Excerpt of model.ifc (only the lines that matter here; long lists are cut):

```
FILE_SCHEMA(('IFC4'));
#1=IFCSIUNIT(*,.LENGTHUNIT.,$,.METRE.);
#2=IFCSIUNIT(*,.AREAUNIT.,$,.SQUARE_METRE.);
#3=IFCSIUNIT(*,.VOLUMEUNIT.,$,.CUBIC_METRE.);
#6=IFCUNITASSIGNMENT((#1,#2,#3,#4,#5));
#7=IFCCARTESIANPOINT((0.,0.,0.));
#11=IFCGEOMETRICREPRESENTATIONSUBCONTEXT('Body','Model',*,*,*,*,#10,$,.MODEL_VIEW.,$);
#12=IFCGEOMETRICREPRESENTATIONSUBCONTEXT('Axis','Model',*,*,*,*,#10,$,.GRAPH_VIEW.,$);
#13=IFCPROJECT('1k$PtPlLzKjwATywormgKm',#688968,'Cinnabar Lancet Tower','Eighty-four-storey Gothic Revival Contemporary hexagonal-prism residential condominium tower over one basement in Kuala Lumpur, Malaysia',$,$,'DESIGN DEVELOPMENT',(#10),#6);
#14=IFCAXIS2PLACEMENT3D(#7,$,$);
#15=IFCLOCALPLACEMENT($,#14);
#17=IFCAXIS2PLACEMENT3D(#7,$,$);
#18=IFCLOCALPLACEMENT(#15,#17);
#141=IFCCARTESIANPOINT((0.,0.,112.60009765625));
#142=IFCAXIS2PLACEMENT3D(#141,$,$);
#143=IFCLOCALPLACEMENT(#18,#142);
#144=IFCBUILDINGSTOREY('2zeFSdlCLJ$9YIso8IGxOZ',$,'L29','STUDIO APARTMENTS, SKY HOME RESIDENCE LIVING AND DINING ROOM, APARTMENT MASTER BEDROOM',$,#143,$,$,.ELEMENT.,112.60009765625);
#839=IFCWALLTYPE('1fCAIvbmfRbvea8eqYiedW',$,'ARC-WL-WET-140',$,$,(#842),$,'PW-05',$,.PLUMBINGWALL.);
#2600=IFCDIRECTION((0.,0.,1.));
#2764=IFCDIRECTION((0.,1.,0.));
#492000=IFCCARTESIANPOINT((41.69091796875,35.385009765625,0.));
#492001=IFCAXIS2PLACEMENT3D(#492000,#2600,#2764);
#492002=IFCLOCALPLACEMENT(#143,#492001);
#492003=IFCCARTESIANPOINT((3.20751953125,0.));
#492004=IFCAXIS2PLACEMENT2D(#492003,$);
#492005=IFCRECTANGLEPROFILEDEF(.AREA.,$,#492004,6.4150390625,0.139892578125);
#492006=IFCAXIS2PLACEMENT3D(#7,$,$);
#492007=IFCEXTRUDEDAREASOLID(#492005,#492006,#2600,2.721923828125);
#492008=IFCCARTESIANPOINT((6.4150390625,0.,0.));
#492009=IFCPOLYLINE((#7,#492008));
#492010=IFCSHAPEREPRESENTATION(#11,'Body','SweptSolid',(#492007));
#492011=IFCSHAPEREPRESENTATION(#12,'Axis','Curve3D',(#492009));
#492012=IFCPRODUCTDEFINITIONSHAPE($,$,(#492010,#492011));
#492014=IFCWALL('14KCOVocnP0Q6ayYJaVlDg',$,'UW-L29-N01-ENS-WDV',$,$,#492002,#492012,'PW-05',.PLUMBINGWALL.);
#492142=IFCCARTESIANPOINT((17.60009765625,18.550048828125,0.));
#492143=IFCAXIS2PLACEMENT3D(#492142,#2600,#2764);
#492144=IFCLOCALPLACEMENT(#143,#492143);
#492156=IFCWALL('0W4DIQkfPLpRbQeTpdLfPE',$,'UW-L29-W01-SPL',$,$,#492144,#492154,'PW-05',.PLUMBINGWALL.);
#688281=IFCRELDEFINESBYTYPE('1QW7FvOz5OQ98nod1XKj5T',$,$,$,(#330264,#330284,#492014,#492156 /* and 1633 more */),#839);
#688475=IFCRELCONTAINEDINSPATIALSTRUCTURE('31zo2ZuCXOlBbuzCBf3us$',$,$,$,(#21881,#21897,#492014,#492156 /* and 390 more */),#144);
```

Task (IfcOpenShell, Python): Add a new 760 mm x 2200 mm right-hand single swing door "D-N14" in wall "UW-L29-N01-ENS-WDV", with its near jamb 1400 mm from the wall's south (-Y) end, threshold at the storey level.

```python
import numpy as np
import ifcopenshell
import ifcopenshell.api.feature
import ifcopenshell.api.geometry
import ifcopenshell.api.root
import ifcopenshell.api.spatial
import ifcopenshell.geom
import ifcopenshell.util.element
import ifcopenshell.util.placement
import ifcopenshell.util.representation
import ifcopenshell.util.shape
import ifcopenshell.util.unit

model = ifcopenshell.open("model.ifc")
unit_scale = ifcopenshell.util.unit.calculate_unit_scale(model)
settings = ifcopenshell.geom.settings()


def volume(element):
    """Net volume in cubic metres, openings subtracted."""
    shape = ifcopenshell.geom.create_shape(settings, element)
    return ifcopenshell.util.shape.get_volume(shape.geometry)


wall = model.by_guid("14KCOVocnP0Q6ayYJaVlDg")
storey = ifcopenshell.util.element.get_container(wall, ifc_class="IfcBuildingStorey")
context = ifcopenshell.util.representation.get_context(model, "Model", "Body", "MODEL_VIEW")
before = volume(wall)

width, height, from_end, sill = 0.76, 2.2, 1.4, 0.0  # metres

# The wall runs along its own X axis, and the end named is its -X end.
wall_shape = ifcopenshell.geom.create_shape(settings, wall)
x, y, z = ifcopenshell.util.shape.get_vertices(wall_shape.geometry).T
start = x.min() + from_end
face, thickness = float(y.min()), float(y.max() - y.min())
wall_matrix = ifcopenshell.util.placement.get_local_placement(wall.ObjectPlacement)
level = ifcopenshell.util.placement.get_local_placement(storey.ObjectPlacement)[2, 3]


def in_wall(x, y):
    """Placement at x, y metres in the wall's axes, at sill height."""
    matrix = wall_matrix.copy()
    matrix[:, 3] = wall_matrix @ np.array([x / unit_scale, y / unit_scale, 0.0, 1.0])
    matrix[2, 3] = level + sill / unit_scale
    return matrix


# Opening: a box that overshoots both wall faces by 50 mm.
opening = ifcopenshell.api.root.create_entity(model, ifc_class="IfcOpeningElement", predefined_type="OPENING")
box = ifcopenshell.api.geometry.add_wall_representation(
    model, context=context, length=width, height=height, thickness=thickness + 0.1
)
ifcopenshell.api.geometry.assign_representation(model, product=opening, representation=box)
ifcopenshell.api.geometry.edit_object_placement(model, product=opening, matrix=in_wall(start, face - 0.05), is_si=False)
ifcopenshell.api.feature.add_feature(model, feature=opening, element=wall)

door = ifcopenshell.api.root.create_entity(model, ifc_class="IfcDoor", name="D-N14", predefined_type="DOOR")
door.OverallWidth, door.OverallHeight = width / unit_scale, height / unit_scale
door.OperationType = "SINGLE_SWING_RIGHT"
body = ifcopenshell.api.geometry.add_door_representation(
    model,
    context=context,
    overall_width=door.OverallWidth,
    overall_height=door.OverallHeight,
    operation_type="SINGLE_SWING_RIGHT",
    lining_properties={"LiningDepth": thickness / unit_scale, "ThresholdDepth": thickness / unit_scale},
)
ifcopenshell.api.geometry.assign_representation(model, product=door, representation=body)
ifcopenshell.api.spatial.assign_container(model, products=[door], relating_structure=storey)
ifcopenshell.api.feature.add_filling(model, opening=opening, element=door)

# The lining spans the wall, so the door starts at the wall face.
ifcopenshell.api.geometry.edit_object_placement(model, product=door, matrix=in_wall(start, face), is_si=False)

after = volume(wall)

print(f"wall volume {before:.3f} -> {after:.3f} m3")

model.write("model-out.ifc")
```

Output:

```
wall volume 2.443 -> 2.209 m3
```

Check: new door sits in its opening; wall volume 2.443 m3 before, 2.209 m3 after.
